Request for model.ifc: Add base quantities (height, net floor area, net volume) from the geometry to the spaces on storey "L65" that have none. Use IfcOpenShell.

First a look at what the model holds.

```python
import ifcopenshell
import ifcopenshell.util.element
import ifcopenshell.util.unit

model = ifcopenshell.open("model.ifc")
print(model.schema)
for unit_type in ("LENGTHUNIT", "AREAUNIT", "VOLUMEUNIT"):
    print(unit_type, ifcopenshell.util.unit.calculate_unit_scale(model, unit_type))
storey = next(s for s in model.by_type("IfcBuildingStorey") if s.Name == "L65")
spaces = [e for e in ifcopenshell.util.element.get_decomposition(storey) if e.is_a("IfcSpace")]
for e in sorted(spaces, key=lambda e: e.id()):
    print(e.id(), e.is_a(), e.Name, list(ifcopenshell.util.element.get_psets(e, qtos_only=True)), sep=" | ")
```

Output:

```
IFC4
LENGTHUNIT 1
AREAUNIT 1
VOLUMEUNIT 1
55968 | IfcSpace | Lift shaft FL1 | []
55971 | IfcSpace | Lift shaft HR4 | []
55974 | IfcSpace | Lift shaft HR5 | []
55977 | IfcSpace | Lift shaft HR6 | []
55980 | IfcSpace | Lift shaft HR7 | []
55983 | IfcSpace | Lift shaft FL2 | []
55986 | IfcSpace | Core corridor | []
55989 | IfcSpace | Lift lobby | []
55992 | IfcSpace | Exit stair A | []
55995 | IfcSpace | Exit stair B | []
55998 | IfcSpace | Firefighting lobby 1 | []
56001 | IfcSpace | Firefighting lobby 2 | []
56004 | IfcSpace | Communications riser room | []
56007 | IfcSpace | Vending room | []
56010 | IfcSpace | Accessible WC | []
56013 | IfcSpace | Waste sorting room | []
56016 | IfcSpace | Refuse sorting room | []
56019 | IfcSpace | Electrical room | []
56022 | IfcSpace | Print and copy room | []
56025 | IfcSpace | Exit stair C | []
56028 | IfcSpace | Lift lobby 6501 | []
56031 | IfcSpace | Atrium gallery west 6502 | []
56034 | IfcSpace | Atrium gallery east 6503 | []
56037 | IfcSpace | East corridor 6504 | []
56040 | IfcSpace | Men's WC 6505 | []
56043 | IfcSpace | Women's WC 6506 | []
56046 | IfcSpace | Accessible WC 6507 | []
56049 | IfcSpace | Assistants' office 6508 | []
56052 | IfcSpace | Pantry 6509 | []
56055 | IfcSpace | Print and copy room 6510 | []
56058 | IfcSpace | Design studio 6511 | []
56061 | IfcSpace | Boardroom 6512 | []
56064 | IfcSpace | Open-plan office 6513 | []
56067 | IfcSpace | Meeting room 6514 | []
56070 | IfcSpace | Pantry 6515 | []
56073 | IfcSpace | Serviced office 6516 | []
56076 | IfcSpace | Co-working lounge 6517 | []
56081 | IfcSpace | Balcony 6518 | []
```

```python
import ifcopenshell
import ifcopenshell.api.pset
import ifcopenshell.geom
import ifcopenshell.util.element
import ifcopenshell.util.shape
import ifcopenshell.util.unit

model = ifcopenshell.open("model.ifc")
unit_scale = ifcopenshell.util.unit.calculate_unit_scale(model)
area_scale = ifcopenshell.util.unit.calculate_unit_scale(model, "AREAUNIT")
volume_scale = ifcopenshell.util.unit.calculate_unit_scale(model, "VOLUMEUNIT")
settings = ifcopenshell.geom.settings()

storey = next(s for s in model.by_type("IfcBuildingStorey") if s.Name == "L65")
spaces = [e for e in ifcopenshell.util.element.get_decomposition(storey) if e.is_a("IfcSpace")]

for e in sorted(spaces, key=lambda e: e.id()):
    if ifcopenshell.util.element.get_psets(e, qtos_only=True, should_inherit=False):
        continue
    # Geometry comes back in metres, in the element's own axes.
    shape = ifcopenshell.geom.create_shape(settings, e)
    values = {
        "Height": ifcopenshell.util.shape.get_z(shape.geometry) / unit_scale,
        "NetFloorArea": ifcopenshell.util.shape.get_footprint_area(shape.geometry) / area_scale,
        "NetVolume": ifcopenshell.util.shape.get_volume(shape.geometry) / volume_scale,
    }
    qto = ifcopenshell.api.pset.add_qto(model, product=e, name="Qto_SpaceBaseQuantities")
    ifcopenshell.api.pset.edit_qto(model, qto=qto, properties=values)
    print(e.id(), {k: round(v, 3) for k, v in values.items()})

model.write("model_edited.ifc")
```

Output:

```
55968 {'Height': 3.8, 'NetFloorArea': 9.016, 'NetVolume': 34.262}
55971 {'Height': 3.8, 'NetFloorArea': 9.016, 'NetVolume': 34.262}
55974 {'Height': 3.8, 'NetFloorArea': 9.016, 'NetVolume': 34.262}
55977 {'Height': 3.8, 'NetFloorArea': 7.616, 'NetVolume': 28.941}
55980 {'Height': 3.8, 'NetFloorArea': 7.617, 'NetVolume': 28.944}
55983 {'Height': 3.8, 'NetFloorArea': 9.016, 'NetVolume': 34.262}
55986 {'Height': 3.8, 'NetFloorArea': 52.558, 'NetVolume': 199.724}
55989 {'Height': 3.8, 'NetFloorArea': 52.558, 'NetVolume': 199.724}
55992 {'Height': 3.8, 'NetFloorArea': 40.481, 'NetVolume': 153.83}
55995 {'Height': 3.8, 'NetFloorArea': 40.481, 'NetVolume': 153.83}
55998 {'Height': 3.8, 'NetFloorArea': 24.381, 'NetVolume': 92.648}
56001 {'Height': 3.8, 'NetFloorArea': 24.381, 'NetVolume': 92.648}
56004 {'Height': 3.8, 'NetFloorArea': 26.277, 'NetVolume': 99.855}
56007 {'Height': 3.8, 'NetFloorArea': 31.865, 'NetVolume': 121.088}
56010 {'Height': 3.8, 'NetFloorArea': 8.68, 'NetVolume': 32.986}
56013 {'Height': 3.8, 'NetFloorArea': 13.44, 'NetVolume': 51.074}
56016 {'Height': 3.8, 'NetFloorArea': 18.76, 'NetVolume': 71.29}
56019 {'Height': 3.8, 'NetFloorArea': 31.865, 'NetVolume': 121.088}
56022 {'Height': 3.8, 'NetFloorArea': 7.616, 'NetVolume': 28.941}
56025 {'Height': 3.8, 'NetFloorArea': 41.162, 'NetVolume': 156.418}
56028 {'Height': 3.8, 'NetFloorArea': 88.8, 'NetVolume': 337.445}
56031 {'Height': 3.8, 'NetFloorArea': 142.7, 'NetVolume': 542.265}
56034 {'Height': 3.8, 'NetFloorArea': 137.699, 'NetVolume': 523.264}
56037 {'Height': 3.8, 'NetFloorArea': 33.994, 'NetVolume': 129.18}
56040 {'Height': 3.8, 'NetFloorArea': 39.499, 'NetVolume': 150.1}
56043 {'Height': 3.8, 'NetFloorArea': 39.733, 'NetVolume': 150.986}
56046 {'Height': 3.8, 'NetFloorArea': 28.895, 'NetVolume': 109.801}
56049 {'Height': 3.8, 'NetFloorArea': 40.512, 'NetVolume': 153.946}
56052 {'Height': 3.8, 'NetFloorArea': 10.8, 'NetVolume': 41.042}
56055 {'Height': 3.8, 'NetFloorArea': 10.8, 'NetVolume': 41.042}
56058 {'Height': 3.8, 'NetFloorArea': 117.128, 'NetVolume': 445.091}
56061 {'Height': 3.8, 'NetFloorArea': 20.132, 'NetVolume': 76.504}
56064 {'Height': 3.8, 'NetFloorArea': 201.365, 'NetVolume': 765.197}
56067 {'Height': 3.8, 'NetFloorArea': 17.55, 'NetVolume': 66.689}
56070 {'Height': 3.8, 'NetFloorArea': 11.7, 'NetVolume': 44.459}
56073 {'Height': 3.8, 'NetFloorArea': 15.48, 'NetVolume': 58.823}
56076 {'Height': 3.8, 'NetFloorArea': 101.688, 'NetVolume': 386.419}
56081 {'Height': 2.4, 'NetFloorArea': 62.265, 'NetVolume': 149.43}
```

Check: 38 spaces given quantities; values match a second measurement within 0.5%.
